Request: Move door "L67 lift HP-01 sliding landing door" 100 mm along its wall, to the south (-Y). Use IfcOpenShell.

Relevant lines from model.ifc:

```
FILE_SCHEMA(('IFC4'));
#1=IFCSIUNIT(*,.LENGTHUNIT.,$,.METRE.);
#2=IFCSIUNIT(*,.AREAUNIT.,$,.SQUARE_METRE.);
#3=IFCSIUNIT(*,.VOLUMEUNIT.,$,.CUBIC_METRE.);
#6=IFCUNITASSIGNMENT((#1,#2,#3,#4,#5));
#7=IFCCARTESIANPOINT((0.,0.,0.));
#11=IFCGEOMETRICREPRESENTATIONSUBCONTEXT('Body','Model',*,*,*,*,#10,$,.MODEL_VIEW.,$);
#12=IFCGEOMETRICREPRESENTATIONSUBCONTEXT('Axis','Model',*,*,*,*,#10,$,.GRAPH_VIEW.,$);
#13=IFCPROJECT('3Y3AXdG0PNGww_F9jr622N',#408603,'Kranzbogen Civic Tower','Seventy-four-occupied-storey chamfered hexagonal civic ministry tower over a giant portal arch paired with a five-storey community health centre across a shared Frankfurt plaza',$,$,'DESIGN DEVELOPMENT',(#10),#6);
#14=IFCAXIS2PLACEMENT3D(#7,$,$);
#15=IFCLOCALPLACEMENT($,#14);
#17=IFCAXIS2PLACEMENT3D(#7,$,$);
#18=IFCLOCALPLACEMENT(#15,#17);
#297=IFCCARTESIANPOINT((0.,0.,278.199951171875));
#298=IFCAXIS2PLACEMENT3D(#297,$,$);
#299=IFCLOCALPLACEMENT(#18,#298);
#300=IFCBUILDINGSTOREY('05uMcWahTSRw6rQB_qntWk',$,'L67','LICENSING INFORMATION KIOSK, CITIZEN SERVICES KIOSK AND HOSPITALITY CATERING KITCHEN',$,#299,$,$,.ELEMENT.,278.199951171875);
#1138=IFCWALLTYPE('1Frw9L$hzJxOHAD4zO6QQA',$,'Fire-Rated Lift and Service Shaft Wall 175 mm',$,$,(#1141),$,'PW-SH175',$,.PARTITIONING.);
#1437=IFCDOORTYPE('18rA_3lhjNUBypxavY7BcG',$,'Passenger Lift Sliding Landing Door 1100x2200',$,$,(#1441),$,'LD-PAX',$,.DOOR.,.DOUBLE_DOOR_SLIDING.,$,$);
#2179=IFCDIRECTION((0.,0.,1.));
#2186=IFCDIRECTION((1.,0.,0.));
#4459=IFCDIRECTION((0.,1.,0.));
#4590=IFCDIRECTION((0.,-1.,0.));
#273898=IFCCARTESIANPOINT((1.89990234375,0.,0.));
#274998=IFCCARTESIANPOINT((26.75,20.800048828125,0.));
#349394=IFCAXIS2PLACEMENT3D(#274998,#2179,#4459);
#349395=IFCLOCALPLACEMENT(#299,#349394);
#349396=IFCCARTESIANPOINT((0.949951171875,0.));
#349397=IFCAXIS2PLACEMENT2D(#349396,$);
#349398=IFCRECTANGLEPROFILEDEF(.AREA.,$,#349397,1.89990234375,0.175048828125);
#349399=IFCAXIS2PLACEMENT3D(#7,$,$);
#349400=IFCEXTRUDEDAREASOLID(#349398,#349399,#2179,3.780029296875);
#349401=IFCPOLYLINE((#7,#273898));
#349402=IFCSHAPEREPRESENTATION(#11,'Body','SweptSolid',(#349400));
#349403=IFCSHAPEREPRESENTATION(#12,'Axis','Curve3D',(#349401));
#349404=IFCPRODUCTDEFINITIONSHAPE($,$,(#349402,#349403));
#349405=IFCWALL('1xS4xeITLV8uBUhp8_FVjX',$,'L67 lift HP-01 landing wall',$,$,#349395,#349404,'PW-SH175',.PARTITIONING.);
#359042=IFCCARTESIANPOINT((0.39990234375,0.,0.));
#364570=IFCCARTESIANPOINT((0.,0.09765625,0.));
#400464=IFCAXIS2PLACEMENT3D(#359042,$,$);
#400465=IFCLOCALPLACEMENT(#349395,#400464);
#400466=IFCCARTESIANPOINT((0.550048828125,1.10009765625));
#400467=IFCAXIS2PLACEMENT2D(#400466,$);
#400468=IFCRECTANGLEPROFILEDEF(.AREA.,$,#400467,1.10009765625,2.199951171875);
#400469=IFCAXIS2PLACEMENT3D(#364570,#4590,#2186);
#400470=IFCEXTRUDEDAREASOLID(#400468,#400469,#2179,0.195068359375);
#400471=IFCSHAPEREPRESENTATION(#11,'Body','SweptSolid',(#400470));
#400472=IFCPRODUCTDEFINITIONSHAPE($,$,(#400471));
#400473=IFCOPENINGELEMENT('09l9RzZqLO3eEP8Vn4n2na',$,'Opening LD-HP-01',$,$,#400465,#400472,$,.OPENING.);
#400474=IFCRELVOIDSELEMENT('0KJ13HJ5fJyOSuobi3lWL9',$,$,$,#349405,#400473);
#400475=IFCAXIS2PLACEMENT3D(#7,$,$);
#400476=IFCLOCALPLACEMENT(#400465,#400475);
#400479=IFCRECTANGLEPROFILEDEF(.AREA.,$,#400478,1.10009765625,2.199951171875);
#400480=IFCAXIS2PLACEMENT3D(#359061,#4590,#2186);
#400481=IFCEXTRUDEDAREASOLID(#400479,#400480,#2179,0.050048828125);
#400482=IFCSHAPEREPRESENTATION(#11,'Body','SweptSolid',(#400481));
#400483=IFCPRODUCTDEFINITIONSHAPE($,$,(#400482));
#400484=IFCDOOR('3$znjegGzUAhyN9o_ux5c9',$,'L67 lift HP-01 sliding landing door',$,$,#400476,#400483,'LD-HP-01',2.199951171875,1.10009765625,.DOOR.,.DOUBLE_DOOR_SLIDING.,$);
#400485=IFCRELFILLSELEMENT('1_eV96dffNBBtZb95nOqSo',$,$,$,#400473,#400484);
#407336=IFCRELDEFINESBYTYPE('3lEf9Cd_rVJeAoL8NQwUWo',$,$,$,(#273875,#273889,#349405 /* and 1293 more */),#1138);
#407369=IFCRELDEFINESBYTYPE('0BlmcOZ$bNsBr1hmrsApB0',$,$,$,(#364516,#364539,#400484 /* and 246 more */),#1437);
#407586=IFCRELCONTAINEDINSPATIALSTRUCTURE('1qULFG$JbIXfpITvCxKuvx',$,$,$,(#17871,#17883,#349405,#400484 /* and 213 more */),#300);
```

```python
import ifcopenshell
import ifcopenshell.api.geometry
import ifcopenshell.util.placement

model = ifcopenshell.open("model.ifc")

door = model.by_guid("3$znjegGzUAhyN9o_ux5c9")
opening = door.FillsVoids[0].RelatingOpeningElement
wall = opening.VoidsElements[0].RelatingBuildingElement

wall_matrix = ifcopenshell.util.placement.get_local_placement(wall.ObjectPlacement)
shift = wall_matrix[:3, 0] * -0.1
before = ifcopenshell.util.placement.get_local_placement(door.ObjectPlacement)[:3, 3].copy()

# The door is placed relative to its opening, so it follows when the opening moves.
matrix = ifcopenshell.util.placement.get_local_placement(opening.ObjectPlacement)
matrix[:3, 3] += shift
ifcopenshell.api.geometry.edit_object_placement(
    model, product=opening, matrix=matrix, is_si=False, should_transform_children=True
)

after = ifcopenshell.util.placement.get_local_placement(door.ObjectPlacement)[:3, 3]
print("door moved by", (after - before).round(3) + 0.0)

model.write("model_updated.ifc")
```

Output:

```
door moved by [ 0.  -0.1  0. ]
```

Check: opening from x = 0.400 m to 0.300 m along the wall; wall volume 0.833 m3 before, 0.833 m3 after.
